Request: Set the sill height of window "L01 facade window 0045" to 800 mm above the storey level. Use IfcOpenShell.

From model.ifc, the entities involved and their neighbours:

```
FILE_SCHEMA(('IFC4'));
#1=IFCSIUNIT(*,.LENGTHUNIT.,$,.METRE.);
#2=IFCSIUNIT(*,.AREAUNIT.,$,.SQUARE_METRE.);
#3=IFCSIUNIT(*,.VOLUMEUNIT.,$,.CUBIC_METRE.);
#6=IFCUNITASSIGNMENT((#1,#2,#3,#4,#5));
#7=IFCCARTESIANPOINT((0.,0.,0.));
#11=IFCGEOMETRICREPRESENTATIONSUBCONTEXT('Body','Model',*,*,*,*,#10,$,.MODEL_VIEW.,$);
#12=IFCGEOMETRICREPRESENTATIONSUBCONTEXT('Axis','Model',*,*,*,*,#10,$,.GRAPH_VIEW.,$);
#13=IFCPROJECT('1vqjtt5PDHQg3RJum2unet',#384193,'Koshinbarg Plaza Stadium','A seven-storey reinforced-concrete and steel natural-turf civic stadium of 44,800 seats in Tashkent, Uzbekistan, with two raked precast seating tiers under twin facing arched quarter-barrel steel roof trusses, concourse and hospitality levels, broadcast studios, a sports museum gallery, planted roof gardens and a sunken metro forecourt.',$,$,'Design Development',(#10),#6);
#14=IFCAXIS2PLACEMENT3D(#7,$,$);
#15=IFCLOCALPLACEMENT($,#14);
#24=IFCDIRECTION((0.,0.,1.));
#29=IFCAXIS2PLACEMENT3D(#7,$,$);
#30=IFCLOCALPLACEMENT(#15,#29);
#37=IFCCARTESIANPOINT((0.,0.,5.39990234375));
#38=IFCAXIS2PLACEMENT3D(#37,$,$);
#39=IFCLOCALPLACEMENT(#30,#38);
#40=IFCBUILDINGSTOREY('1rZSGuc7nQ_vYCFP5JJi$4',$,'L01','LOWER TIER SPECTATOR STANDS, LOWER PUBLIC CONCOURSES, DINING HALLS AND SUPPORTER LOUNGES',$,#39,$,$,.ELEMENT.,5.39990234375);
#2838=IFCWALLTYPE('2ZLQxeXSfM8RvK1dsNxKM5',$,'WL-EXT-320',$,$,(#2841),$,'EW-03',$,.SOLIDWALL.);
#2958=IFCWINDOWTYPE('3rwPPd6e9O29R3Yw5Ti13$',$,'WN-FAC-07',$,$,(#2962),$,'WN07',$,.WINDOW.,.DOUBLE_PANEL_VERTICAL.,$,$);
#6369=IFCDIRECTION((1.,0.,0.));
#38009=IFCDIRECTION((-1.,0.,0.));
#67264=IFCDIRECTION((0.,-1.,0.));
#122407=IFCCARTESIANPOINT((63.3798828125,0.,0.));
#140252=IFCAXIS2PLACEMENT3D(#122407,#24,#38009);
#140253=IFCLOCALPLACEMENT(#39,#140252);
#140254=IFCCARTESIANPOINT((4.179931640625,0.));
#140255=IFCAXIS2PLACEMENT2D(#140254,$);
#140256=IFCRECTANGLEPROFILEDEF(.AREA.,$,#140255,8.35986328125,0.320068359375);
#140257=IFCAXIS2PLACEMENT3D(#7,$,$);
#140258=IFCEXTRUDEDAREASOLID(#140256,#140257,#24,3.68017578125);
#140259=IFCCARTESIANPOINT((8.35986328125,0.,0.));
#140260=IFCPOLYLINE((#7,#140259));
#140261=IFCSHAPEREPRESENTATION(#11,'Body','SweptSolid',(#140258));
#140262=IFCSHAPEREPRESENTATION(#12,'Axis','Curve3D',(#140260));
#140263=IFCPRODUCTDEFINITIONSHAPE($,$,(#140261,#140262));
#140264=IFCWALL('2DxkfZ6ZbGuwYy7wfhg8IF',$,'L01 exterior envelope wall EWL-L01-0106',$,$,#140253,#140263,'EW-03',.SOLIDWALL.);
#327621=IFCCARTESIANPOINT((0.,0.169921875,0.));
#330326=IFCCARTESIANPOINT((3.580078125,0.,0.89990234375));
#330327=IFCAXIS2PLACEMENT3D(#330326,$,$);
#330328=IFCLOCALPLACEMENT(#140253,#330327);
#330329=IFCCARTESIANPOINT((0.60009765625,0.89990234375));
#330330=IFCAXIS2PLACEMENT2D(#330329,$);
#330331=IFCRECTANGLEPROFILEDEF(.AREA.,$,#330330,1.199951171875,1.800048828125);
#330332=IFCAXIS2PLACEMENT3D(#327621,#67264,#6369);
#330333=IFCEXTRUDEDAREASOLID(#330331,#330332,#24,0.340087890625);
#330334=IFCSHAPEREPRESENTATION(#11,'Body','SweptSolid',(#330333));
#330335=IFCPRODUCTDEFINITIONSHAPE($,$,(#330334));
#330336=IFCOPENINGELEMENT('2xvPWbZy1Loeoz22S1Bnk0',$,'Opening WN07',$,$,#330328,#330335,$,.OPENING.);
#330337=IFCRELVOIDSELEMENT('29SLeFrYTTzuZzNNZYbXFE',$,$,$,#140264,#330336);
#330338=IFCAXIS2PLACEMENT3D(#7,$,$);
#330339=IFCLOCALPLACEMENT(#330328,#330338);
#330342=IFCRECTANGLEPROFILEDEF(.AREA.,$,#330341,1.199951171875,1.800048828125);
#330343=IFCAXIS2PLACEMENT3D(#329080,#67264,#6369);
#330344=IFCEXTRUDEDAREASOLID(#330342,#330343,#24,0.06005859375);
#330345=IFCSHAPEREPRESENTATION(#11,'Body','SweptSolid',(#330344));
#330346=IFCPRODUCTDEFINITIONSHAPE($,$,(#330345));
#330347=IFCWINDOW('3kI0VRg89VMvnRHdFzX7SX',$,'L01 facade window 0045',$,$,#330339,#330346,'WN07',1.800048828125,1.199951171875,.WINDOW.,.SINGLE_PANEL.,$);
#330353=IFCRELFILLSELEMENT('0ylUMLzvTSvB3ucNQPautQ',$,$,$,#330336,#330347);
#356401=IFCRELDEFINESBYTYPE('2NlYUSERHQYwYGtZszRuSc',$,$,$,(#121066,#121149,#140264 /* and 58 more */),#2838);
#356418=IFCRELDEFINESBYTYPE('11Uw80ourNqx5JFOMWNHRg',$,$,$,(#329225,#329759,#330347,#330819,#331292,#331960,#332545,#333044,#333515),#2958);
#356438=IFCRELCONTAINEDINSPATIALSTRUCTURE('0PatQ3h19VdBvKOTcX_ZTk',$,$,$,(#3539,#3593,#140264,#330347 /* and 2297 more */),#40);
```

```python
import numpy as np
import ifcopenshell
import ifcopenshell.api.geometry
import ifcopenshell.geom
import ifcopenshell.util.element
import ifcopenshell.util.placement
import ifcopenshell.util.shape
import ifcopenshell.util.unit

model = ifcopenshell.open("model.ifc")
unit_scale = ifcopenshell.util.unit.calculate_unit_scale(model)

window = model.by_id(330347)
opening = window.FillsVoids[0].RelatingOpeningElement
storey = ifcopenshell.util.element.get_container(window, ifc_class="IfcBuildingStorey")
level = ifcopenshell.util.placement.get_local_placement(storey.ObjectPlacement)[2, 3]

# The opening's origin need not be at the sill, so measure its lowest point.
shape = ifcopenshell.geom.create_shape(ifcopenshell.geom.settings(), opening)
bottom = ifcopenshell.util.shape.get_shape_bottom_elevation(shape, shape.geometry) / unit_scale
dz = level + 0.8 - bottom

shift = np.array([0.0, 0.0, dz])
# The window is placed relative to its opening, so it follows when the opening moves.
matrix = ifcopenshell.util.placement.get_local_placement(opening.ObjectPlacement)
matrix[:3, 3] += shift
ifcopenshell.api.geometry.edit_object_placement(
    model, product=opening, matrix=matrix, is_si=False, should_transform_children=True
)

print(f"moved by {dz * unit_scale:+.3f} m")

model.write("model-out.ifc")
```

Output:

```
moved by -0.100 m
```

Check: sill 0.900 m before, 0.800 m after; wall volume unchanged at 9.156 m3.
